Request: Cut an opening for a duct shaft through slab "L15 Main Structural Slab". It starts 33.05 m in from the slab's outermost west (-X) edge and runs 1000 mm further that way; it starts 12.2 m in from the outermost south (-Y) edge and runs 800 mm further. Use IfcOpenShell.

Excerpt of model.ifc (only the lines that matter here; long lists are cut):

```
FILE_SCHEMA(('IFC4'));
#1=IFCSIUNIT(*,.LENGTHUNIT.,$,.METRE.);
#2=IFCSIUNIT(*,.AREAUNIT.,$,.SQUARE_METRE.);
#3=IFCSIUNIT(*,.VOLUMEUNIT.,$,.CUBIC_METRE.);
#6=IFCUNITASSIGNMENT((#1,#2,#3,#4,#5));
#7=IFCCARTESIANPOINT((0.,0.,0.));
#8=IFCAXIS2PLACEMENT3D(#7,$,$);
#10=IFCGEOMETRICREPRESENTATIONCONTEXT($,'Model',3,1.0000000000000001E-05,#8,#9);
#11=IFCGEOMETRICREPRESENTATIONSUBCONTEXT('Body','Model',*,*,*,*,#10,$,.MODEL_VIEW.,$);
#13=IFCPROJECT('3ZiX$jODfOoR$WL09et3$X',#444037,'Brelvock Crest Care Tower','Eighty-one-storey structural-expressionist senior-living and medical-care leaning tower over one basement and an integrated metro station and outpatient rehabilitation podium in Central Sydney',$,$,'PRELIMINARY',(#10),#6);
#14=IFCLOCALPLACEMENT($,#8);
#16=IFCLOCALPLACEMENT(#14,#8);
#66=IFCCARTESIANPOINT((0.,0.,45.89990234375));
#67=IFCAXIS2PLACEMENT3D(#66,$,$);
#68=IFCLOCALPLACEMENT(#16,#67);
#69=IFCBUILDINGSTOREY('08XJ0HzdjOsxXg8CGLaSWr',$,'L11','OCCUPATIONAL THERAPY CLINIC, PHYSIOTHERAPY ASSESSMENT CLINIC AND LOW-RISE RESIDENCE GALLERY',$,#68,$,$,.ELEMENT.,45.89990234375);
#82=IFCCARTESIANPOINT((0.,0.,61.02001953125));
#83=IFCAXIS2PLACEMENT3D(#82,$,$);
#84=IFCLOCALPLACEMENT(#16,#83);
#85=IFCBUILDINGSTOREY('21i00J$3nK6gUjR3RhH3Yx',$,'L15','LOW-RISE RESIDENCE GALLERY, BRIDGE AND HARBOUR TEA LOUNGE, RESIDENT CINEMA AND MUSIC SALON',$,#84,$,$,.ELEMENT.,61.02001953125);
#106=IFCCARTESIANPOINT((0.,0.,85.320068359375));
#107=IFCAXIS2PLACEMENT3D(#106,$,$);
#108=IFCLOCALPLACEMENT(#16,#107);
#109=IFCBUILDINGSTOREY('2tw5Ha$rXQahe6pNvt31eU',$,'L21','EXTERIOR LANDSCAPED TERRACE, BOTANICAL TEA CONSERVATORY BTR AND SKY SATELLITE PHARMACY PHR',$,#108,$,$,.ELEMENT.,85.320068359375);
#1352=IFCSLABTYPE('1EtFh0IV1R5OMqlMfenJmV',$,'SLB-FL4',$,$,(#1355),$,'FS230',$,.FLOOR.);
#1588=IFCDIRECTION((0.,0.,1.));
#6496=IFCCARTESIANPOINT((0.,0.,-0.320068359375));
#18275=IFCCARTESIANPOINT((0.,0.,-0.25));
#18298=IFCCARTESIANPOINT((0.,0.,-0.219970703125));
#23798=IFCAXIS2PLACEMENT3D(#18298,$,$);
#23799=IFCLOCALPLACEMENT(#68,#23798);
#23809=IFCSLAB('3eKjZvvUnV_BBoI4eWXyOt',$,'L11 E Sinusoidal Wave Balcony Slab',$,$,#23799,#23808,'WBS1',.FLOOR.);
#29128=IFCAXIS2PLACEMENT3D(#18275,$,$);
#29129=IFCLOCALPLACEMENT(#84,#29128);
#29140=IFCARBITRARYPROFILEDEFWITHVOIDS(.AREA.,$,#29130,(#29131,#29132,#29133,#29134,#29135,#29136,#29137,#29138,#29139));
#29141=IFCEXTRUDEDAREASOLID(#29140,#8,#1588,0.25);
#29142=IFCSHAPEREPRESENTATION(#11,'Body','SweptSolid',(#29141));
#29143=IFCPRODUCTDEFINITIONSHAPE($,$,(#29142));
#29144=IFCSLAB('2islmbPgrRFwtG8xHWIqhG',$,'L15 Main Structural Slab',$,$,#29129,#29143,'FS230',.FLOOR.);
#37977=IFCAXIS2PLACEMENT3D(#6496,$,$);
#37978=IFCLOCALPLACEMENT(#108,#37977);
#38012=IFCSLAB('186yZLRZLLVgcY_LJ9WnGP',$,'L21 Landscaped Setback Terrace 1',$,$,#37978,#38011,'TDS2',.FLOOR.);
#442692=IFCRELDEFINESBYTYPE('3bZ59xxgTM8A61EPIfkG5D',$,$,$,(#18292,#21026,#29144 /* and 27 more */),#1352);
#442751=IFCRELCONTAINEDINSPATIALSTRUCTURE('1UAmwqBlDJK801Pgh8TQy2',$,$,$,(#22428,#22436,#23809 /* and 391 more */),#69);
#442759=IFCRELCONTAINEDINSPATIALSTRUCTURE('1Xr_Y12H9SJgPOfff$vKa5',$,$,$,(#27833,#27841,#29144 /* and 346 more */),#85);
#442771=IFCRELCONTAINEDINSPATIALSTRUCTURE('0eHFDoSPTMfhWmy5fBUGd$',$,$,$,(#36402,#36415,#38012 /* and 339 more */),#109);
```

```python
import numpy as np
import ifcopenshell
import ifcopenshell.api.feature
import ifcopenshell.api.geometry
import ifcopenshell.api.root
import ifcopenshell.geom
import ifcopenshell.util.placement
import ifcopenshell.util.representation
import ifcopenshell.util.shape
import ifcopenshell.util.unit

model = ifcopenshell.open("model.ifc")
unit_scale = ifcopenshell.util.unit.calculate_unit_scale(model)
settings = ifcopenshell.geom.settings()


def volume(element):
    """Net volume in cubic metres, openings subtracted."""
    shape = ifcopenshell.geom.create_shape(settings, element)
    return ifcopenshell.util.shape.get_volume(shape.geometry)


slab = model.by_guid("2islmbPgrRFwtG8xHWIqhG")
before = volume(slab)

# Extent in the slab's own axes, in metres. The edges named are its -X and -Y sides.
slab_shape = ifcopenshell.geom.create_shape(settings, slab)
vertices = ifcopenshell.util.shape.get_vertices(slab_shape.geometry)
x_min, y_min, bottom = vertices.min(axis=0)
top = vertices[:, 2].max()

opening = ifcopenshell.api.root.create_entity(model, ifc_class="IfcOpeningElement", name="Duct shaft opening", predefined_type="OPENING")
context = ifcopenshell.util.representation.get_context(model, "Model", "Body", "MODEL_VIEW")
width, depth = 1, 0.8
outline = [(0.0, 0.0), (width, 0.0), (width, depth), (0.0, depth), (0.0, 0.0)]
# Overshoot both faces by 50 mm so the cut is clean.
shape = ifcopenshell.api.geometry.add_slab_representation(
    model, context=context, depth=top - bottom + 0.1, polyline=outline
)
ifcopenshell.api.geometry.assign_representation(model, product=opening, representation=shape)

matrix = ifcopenshell.util.placement.get_local_placement(slab.ObjectPlacement)
matrix[:, 3] = matrix @ np.append(np.array([x_min + 33.05, y_min + 12.2, bottom - 0.05]) / unit_scale, 1.0)
ifcopenshell.api.geometry.edit_object_placement(model, product=opening, matrix=matrix, is_si=False)
ifcopenshell.api.feature.add_feature(model, feature=opening, element=slab)

after = volume(slab)

print(f"slab volume {before:.3f} -> {after:.3f} m3")

model.write("model_v2.ifc")
```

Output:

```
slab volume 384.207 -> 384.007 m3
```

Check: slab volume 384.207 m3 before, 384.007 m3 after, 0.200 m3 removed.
